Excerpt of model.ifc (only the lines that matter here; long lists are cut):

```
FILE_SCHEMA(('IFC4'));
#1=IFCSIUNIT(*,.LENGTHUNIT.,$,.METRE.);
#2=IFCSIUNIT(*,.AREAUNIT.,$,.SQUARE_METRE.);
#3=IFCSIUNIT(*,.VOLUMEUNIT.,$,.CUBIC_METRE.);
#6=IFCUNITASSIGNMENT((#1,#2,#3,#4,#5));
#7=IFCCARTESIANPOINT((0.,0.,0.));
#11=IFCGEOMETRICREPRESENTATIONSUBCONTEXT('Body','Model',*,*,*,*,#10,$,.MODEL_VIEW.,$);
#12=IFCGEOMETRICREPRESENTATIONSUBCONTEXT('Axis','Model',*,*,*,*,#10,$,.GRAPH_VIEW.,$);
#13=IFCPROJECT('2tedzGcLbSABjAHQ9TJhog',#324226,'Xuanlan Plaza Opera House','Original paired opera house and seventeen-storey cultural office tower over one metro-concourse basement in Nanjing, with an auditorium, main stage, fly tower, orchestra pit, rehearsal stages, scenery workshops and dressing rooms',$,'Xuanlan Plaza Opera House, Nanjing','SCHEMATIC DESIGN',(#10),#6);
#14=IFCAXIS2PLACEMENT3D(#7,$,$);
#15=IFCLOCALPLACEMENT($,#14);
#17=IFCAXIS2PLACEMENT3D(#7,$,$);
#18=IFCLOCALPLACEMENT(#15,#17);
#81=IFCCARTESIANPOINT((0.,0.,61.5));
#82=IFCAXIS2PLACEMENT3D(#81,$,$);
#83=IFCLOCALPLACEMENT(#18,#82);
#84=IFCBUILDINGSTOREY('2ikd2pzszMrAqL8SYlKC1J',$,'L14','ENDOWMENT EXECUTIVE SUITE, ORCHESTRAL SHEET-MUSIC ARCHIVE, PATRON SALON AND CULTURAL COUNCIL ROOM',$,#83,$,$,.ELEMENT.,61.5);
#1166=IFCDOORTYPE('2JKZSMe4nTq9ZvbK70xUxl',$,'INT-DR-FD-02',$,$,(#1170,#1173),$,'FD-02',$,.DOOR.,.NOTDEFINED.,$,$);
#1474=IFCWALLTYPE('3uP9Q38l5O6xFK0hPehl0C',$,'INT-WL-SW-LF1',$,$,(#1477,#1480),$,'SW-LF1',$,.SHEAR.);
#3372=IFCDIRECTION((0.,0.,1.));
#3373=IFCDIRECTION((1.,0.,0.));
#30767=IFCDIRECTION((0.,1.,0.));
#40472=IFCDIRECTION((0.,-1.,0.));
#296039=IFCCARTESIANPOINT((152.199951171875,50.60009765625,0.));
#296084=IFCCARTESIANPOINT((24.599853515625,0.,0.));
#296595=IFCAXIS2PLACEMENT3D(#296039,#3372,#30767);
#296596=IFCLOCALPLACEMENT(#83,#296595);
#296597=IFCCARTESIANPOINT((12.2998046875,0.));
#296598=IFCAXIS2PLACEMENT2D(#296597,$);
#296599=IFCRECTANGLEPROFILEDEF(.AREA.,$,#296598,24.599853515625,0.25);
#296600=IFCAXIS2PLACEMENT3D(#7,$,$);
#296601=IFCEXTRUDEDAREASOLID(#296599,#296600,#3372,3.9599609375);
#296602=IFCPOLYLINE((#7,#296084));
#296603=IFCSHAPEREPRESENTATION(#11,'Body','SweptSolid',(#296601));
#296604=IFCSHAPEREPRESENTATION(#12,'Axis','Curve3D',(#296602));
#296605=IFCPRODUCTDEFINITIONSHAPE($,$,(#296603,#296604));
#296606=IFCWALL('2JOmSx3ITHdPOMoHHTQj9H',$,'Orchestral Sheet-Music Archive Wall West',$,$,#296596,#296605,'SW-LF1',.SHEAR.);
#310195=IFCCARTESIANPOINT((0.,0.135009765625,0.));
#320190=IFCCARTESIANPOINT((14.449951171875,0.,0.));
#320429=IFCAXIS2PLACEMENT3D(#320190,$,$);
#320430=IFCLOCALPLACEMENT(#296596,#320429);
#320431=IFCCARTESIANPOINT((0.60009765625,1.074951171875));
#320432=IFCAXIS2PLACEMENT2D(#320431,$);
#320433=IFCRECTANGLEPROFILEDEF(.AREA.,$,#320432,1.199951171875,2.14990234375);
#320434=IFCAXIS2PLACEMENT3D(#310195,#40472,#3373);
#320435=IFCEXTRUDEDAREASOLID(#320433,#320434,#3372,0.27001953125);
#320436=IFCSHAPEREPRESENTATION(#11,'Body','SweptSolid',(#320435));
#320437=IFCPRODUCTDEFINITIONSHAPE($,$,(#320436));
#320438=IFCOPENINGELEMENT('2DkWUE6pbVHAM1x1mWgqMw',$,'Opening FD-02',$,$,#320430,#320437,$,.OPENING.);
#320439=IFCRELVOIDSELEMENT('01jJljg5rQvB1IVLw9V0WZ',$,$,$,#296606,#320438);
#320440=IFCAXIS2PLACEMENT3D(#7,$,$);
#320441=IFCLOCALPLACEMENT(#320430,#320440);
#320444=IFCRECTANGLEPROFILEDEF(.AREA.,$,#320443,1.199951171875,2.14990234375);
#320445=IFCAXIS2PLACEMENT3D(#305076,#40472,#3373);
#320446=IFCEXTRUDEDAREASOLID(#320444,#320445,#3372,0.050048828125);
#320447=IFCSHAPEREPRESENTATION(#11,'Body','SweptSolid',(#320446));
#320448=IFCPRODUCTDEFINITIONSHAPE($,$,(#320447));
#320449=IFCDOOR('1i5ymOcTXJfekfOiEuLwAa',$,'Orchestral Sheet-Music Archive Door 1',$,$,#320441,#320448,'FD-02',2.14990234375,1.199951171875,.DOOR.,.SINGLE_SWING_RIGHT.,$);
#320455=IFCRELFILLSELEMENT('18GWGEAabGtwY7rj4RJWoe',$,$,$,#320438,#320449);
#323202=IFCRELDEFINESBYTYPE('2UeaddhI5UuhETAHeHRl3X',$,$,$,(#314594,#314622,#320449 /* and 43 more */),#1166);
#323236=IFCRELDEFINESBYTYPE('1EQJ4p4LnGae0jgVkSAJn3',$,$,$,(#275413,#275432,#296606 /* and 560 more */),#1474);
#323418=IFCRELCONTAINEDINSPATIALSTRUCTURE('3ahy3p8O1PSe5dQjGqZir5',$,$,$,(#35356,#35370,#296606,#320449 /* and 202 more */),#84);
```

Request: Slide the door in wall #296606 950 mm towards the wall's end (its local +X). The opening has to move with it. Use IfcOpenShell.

```python
import ifcopenshell
import ifcopenshell.api.geometry
import ifcopenshell.util.placement
import ifcopenshell.util.unit

model = ifcopenshell.open("model.ifc")
unit_scale = ifcopenshell.util.unit.calculate_unit_scale(model)

door = model.by_guid("1i5ymOcTXJfekfOiEuLwAa")
opening = door.FillsVoids[0].RelatingOpeningElement
wall = opening.VoidsElements[0].RelatingBuildingElement

wall_matrix = ifcopenshell.util.placement.get_local_placement(wall.ObjectPlacement)
shift = wall_matrix[:3, 0] * 0.95 / unit_scale
before = ifcopenshell.util.placement.get_local_placement(door.ObjectPlacement)[:3, 3].copy()

# The door is placed relative to its opening, so it follows when the opening moves.
matrix = ifcopenshell.util.placement.get_local_placement(opening.ObjectPlacement)
matrix[:3, 3] += shift
ifcopenshell.api.geometry.edit_object_placement(
    model, product=opening, matrix=matrix, is_si=False, should_transform_children=True
)

after = ifcopenshell.util.placement.get_local_placement(door.ObjectPlacement)[:3, 3]
print("door moved by", (after - before).round(3) + 0.0)

model.write("model_v2.ifc")
```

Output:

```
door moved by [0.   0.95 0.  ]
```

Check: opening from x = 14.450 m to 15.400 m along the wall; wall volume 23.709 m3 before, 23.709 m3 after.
